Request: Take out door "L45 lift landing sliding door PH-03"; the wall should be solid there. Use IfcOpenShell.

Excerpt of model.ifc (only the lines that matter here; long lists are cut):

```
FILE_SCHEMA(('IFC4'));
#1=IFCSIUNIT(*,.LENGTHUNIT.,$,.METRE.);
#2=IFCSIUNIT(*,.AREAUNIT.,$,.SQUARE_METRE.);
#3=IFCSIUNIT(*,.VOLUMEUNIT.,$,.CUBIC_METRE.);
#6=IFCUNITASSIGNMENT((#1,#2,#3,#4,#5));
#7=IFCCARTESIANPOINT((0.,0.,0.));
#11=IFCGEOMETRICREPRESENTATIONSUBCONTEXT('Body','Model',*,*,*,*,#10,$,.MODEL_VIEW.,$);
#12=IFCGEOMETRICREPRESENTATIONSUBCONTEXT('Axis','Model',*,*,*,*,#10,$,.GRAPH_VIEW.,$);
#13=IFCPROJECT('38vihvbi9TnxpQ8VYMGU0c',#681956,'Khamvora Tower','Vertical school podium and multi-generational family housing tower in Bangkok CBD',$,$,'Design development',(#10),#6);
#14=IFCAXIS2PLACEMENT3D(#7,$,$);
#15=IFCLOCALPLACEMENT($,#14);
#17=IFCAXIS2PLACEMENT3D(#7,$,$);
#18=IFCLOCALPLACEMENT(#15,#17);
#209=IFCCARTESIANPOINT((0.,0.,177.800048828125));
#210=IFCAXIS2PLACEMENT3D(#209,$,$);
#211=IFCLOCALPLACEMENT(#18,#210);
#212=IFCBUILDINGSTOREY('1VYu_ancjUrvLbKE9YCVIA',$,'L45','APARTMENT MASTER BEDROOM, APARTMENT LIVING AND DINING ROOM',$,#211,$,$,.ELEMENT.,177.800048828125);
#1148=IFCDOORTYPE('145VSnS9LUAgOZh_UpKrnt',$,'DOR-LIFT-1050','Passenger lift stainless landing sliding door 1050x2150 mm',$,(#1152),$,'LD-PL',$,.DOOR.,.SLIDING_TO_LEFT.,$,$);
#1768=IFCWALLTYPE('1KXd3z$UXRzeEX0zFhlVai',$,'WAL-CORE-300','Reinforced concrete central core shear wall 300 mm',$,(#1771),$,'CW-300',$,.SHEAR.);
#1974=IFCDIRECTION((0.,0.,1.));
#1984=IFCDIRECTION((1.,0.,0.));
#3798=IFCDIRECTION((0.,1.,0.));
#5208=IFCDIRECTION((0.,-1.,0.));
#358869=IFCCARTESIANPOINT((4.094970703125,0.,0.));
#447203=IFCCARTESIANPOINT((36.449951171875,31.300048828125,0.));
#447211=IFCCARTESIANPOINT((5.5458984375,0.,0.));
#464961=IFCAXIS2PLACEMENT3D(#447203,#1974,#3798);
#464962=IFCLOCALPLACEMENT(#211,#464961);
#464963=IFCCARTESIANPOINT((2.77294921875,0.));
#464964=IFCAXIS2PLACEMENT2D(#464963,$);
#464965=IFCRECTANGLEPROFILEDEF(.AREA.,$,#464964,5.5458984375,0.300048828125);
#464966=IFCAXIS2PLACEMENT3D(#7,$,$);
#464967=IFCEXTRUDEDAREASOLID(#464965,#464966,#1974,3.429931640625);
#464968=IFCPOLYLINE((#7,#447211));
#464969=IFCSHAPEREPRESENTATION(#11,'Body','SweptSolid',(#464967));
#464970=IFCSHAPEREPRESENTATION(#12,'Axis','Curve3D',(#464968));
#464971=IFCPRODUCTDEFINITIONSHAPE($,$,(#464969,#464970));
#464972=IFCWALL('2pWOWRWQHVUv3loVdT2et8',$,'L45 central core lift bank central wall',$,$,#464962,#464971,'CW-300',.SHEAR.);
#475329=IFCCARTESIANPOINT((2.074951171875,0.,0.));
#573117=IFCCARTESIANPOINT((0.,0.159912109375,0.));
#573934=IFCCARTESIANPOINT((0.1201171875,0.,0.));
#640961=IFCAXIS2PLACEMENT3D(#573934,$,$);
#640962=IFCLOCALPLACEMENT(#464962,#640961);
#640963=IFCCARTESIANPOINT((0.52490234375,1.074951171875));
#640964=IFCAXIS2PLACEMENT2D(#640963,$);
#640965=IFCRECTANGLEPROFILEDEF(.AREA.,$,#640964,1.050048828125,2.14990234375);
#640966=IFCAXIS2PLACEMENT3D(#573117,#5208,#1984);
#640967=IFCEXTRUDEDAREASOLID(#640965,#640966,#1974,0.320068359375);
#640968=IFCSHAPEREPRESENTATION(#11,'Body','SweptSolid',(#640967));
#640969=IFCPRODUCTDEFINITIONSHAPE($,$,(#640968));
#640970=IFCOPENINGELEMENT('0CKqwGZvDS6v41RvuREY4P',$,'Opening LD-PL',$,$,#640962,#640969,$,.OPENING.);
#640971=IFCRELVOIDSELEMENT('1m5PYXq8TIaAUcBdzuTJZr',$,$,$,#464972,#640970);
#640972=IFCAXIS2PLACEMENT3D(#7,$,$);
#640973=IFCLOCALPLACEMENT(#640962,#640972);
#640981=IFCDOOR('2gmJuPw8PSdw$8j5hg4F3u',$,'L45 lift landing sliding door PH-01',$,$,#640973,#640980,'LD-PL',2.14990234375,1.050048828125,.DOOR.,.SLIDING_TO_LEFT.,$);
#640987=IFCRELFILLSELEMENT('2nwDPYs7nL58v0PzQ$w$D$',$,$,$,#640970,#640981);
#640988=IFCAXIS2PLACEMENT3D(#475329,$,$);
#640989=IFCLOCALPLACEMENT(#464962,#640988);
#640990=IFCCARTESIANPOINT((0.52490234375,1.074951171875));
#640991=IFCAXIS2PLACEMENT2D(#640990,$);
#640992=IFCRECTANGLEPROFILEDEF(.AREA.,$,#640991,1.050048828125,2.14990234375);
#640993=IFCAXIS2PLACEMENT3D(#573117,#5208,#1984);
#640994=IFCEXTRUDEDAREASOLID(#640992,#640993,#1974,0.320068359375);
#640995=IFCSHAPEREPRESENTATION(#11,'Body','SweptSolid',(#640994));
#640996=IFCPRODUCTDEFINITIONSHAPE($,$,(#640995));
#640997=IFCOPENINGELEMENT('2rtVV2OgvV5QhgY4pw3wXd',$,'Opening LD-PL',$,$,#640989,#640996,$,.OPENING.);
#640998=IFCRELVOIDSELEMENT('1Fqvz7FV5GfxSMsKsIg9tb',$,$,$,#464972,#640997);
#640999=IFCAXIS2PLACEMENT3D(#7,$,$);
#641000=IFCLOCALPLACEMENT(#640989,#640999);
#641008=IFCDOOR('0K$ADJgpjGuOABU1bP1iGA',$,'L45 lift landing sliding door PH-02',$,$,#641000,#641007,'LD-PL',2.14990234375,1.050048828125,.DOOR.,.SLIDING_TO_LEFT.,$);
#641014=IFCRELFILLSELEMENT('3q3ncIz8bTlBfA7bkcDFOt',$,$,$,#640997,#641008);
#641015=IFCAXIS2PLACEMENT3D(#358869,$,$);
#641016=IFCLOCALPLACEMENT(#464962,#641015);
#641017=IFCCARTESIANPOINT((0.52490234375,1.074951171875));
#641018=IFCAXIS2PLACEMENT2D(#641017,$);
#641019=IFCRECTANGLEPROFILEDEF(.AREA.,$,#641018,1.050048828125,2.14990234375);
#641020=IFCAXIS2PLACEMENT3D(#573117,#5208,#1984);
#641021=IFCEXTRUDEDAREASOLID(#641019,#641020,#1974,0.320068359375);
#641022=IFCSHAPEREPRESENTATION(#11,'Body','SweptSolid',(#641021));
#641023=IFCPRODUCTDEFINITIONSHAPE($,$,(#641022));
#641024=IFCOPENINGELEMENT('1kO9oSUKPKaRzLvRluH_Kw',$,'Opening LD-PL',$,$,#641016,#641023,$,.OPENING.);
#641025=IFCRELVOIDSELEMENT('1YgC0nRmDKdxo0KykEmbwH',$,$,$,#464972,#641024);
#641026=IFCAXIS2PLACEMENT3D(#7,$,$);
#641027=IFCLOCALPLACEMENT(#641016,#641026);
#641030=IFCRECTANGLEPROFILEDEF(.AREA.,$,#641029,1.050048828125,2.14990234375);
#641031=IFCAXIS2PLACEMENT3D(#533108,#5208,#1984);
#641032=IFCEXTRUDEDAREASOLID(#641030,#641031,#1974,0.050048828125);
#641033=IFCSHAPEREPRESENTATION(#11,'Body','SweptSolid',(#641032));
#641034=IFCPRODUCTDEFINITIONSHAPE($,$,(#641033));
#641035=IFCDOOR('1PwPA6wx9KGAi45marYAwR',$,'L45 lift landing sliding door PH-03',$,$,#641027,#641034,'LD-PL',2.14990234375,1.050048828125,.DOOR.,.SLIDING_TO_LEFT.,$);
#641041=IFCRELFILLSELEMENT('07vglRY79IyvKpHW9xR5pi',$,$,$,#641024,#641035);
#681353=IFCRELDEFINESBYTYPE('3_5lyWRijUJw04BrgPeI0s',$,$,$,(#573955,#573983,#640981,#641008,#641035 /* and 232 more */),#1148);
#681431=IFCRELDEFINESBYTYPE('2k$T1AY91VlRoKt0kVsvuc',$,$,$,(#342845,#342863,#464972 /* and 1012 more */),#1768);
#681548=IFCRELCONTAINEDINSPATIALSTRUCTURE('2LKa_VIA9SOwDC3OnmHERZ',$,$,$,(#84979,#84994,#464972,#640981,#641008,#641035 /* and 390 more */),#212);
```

```python
import ifcopenshell
import ifcopenshell.api.feature
import ifcopenshell.api.root
import ifcopenshell.geom
import ifcopenshell.util.shape

model = ifcopenshell.open("model.ifc")
settings = ifcopenshell.geom.settings()


def volume(element):
    """Net volume in cubic metres, openings subtracted."""
    shape = ifcopenshell.geom.create_shape(settings, element)
    return ifcopenshell.util.shape.get_volume(shape.geometry)


door = model.by_id(641035)
opening = door.FillsVoids[0].RelatingOpeningElement
wall = opening.VoidsElements[0].RelatingBuildingElement
before = volume(wall)

ifcopenshell.api.root.remove_product(model, product=door)
ifcopenshell.api.feature.remove_feature(model, feature=opening)

after = volume(wall)

print(f"wall volume {before:.3f} -> {after:.3f} m3")

model.write("model_edited.ifc")
```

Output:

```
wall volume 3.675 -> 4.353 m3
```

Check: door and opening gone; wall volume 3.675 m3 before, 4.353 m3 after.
